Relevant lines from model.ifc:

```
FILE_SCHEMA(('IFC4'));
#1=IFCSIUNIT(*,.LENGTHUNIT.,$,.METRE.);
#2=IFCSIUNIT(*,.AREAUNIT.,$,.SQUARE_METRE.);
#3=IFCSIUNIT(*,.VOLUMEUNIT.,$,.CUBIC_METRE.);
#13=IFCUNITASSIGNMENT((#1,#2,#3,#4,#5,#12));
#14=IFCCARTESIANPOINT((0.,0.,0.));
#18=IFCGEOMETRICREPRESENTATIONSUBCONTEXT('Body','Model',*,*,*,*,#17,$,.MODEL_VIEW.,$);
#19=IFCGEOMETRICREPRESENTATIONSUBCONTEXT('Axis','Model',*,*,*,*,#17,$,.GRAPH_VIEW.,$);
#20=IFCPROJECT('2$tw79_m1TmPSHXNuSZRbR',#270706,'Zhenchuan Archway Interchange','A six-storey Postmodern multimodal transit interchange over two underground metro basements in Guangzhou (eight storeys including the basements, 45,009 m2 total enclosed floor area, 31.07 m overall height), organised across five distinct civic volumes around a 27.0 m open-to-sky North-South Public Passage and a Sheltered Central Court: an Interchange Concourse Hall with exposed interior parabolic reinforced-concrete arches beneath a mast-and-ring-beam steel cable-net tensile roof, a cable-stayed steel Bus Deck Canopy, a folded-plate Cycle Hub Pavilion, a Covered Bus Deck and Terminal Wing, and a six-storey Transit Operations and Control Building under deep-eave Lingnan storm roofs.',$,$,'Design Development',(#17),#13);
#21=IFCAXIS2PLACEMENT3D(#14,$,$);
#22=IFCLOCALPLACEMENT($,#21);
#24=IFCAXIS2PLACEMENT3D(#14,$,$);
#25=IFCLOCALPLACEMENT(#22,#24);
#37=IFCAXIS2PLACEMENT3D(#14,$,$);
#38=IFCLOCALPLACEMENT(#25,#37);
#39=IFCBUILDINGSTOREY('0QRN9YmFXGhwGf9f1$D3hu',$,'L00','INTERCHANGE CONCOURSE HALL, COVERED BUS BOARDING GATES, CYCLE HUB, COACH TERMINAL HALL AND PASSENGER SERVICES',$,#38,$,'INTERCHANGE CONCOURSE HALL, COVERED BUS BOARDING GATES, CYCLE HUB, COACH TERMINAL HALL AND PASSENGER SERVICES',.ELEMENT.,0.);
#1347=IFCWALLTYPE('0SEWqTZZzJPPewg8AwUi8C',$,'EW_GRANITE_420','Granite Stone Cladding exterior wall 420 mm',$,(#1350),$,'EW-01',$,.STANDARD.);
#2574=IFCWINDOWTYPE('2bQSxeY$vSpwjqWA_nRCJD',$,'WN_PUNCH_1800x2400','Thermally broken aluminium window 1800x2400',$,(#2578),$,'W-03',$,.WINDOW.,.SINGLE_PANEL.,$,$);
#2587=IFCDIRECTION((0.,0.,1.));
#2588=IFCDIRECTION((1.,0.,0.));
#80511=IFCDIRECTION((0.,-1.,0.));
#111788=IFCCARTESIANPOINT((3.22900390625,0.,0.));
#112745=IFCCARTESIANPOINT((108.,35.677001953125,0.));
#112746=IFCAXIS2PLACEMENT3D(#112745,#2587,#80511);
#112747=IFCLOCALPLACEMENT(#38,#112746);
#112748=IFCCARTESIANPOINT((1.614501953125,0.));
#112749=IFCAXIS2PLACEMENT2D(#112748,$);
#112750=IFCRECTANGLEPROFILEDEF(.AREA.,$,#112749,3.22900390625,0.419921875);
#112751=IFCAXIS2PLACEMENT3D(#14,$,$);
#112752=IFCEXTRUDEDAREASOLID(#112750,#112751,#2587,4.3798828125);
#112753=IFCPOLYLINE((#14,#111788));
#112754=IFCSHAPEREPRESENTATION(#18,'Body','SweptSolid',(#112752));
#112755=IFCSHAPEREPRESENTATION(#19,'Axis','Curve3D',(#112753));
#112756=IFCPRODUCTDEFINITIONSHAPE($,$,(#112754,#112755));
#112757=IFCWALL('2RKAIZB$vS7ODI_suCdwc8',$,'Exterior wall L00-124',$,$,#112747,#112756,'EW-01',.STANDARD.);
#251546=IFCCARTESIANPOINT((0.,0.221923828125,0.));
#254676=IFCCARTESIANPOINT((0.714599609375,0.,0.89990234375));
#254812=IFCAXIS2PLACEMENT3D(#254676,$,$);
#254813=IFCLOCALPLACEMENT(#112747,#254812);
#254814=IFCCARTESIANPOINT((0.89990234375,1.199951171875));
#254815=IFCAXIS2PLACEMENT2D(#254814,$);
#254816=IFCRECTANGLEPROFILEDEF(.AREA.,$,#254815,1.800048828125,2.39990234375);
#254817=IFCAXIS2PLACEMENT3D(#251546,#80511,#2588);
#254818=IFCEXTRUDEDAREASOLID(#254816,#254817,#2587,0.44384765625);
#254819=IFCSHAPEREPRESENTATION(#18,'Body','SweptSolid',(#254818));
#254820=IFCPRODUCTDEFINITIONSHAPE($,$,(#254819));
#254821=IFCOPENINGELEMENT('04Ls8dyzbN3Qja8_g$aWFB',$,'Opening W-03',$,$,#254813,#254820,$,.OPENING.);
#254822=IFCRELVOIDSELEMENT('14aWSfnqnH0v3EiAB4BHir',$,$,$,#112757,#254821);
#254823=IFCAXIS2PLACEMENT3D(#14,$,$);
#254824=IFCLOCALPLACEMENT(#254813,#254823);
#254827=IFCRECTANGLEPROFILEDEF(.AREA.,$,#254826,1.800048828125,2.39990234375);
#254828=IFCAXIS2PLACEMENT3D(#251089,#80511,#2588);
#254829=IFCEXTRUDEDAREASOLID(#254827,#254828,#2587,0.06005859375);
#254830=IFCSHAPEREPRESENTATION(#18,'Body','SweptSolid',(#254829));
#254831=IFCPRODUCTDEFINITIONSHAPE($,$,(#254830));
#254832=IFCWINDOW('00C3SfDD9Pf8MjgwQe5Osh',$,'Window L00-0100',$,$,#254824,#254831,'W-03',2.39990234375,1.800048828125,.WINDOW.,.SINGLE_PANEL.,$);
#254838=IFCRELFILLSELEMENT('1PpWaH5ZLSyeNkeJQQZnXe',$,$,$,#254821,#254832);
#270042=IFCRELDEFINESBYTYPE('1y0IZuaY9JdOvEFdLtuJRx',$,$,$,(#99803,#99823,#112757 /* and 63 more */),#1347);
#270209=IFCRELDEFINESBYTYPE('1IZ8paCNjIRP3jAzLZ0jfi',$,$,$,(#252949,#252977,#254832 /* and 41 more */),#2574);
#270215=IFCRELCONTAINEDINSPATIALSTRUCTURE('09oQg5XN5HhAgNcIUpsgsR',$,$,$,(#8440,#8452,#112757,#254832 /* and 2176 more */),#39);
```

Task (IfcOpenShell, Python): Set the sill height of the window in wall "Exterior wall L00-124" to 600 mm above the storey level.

```python
import numpy as np
import ifcopenshell
import ifcopenshell.api.geometry
import ifcopenshell.geom
import ifcopenshell.util.element
import ifcopenshell.util.placement
import ifcopenshell.util.shape
import ifcopenshell.util.unit

model = ifcopenshell.open("model.ifc")
unit_scale = ifcopenshell.util.unit.calculate_unit_scale(model)

window = model.by_guid("00C3SfDD9Pf8MjgwQe5Osh")
opening = window.FillsVoids[0].RelatingOpeningElement
storey = ifcopenshell.util.element.get_container(window, ifc_class="IfcBuildingStorey")
level = ifcopenshell.util.placement.get_local_placement(storey.ObjectPlacement)[2, 3]

# The opening's origin need not be at the sill, so measure its lowest point.
shape = ifcopenshell.geom.create_shape(ifcopenshell.geom.settings(), opening)
bottom = ifcopenshell.util.shape.get_shape_bottom_elevation(shape, shape.geometry) / unit_scale
dz = level + 0.6 / unit_scale - bottom

shift = np.array([0.0, 0.0, dz])
# The window is placed relative to its opening, so it follows when the opening moves.
matrix = ifcopenshell.util.placement.get_local_placement(opening.ObjectPlacement)
matrix[:3, 3] += shift
ifcopenshell.api.geometry.edit_object_placement(
    model, product=opening, matrix=matrix, is_si=False, should_transform_children=True
)

print(f"moved by {dz * unit_scale:+.3f} m")

model.write("model-out.ifc")
```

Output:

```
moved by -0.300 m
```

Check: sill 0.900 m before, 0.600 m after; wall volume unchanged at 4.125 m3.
